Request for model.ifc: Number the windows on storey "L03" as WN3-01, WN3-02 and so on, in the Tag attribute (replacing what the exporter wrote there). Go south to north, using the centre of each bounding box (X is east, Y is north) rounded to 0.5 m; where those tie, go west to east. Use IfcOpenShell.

First a look at what the model holds.

```python
import ifcopenshell
import ifcopenshell.util.element
import ifcopenshell.util.placement

model = ifcopenshell.open("model.ifc")
print(model.schema)
storey = next(s for s in model.by_type("IfcBuildingStorey") if s.Name == "L03")
windows = [e for e in ifcopenshell.util.element.get_decomposition(storey) if e.is_a("IfcWindow")]
for e in sorted(windows, key=lambda e: e.id()):
    origin = ifcopenshell.util.placement.get_local_placement(e.ObjectPlacement)[:3, 3]
    print(e.id(), e.Tag, e.Name, origin.round(2) + 0.0, sep=" | ")
```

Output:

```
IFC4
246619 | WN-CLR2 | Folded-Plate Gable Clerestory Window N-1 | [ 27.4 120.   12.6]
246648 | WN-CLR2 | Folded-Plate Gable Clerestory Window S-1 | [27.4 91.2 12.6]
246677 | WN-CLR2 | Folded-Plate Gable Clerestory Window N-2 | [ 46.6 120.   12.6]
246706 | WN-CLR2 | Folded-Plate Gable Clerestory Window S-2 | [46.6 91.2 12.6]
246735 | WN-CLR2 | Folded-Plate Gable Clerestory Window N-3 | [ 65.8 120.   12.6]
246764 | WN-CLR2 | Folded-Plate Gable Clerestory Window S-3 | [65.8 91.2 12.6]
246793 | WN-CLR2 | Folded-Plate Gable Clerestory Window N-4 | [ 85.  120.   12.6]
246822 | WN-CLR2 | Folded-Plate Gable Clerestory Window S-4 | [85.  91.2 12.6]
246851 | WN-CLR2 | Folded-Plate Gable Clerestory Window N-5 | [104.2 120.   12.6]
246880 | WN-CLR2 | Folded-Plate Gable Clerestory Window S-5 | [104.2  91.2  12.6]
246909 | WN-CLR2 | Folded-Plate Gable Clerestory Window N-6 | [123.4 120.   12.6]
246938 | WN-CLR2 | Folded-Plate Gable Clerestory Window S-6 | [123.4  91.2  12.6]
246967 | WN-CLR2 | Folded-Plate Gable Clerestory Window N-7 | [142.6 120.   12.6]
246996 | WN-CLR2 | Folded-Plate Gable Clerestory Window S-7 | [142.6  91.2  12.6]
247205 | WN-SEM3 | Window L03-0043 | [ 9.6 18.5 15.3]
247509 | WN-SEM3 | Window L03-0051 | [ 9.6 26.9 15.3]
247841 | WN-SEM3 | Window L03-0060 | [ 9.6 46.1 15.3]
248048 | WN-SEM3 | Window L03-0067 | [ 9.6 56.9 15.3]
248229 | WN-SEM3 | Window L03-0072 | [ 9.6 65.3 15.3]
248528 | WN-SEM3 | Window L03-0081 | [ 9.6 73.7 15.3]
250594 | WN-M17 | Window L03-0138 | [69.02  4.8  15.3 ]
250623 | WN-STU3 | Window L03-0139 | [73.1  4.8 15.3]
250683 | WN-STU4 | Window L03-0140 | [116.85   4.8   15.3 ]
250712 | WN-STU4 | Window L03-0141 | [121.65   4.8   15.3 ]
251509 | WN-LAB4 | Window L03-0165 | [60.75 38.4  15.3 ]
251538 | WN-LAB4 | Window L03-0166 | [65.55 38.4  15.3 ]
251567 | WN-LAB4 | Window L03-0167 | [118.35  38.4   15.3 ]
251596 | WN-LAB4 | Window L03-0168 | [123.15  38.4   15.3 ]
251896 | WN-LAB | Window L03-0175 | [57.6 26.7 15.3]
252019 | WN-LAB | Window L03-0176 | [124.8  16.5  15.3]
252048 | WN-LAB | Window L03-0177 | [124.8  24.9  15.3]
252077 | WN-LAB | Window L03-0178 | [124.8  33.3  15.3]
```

```python
import ifcopenshell
import ifcopenshell.geom
import ifcopenshell.util.element
import ifcopenshell.util.shape

model = ifcopenshell.open("model.ifc")
settings = ifcopenshell.geom.settings()
settings.set("use-world-coords", True)


def centre(element):
    shape = ifcopenshell.geom.create_shape(settings, element)
    return ifcopenshell.util.shape.get_bbox_centroid(shape.geometry)


storey = next(s for s in model.by_type("IfcBuildingStorey") if s.Name == "L03")
windows = [e for e in ifcopenshell.util.element.get_decomposition(storey) if e.is_a("IfcWindow")]

# Insertion points can sit at a corner or the storey origin, so sort by the geometry (in metres).
centres = {e: centre(e) for e in windows}
windows.sort(key=lambda e: (round(centres[e][1] / 0.5), centres[e][0]))

for i, e in enumerate(windows, start=1):
    number = f"WN3-{i:02d}"
    e.Tag = number
    print(e.id(), number)

model.write("model_rev.ifc")
```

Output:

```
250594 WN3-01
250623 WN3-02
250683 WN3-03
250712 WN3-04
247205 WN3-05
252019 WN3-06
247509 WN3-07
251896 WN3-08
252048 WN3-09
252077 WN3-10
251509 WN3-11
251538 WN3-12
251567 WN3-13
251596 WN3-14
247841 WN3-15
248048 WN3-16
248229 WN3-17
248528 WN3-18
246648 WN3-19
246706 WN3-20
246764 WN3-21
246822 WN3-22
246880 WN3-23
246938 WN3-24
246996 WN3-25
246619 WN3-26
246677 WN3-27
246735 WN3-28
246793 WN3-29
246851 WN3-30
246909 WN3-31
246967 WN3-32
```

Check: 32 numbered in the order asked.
